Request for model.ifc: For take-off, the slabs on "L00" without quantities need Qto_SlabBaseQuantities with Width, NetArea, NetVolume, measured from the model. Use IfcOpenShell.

First a look at what the model holds.

```python
import ifcopenshell
import ifcopenshell.util.element
import ifcopenshell.util.unit

model = ifcopenshell.open("model.ifc")
print(model.schema)
for unit_type in ("LENGTHUNIT", "AREAUNIT", "VOLUMEUNIT"):
    print(unit_type, ifcopenshell.util.unit.calculate_unit_scale(model, unit_type))
storey = next(s for s in model.by_type("IfcBuildingStorey") if s.Name == "L00")
slabs = [e for e in ifcopenshell.util.element.get_decomposition(storey) if e.is_a("IfcSlab")]
for e in sorted(slabs, key=lambda e: e.id()):
    print(e.id(), e.is_a(), e.Name, list(ifcopenshell.util.element.get_psets(e, qtos_only=True)), sep=" | ")
```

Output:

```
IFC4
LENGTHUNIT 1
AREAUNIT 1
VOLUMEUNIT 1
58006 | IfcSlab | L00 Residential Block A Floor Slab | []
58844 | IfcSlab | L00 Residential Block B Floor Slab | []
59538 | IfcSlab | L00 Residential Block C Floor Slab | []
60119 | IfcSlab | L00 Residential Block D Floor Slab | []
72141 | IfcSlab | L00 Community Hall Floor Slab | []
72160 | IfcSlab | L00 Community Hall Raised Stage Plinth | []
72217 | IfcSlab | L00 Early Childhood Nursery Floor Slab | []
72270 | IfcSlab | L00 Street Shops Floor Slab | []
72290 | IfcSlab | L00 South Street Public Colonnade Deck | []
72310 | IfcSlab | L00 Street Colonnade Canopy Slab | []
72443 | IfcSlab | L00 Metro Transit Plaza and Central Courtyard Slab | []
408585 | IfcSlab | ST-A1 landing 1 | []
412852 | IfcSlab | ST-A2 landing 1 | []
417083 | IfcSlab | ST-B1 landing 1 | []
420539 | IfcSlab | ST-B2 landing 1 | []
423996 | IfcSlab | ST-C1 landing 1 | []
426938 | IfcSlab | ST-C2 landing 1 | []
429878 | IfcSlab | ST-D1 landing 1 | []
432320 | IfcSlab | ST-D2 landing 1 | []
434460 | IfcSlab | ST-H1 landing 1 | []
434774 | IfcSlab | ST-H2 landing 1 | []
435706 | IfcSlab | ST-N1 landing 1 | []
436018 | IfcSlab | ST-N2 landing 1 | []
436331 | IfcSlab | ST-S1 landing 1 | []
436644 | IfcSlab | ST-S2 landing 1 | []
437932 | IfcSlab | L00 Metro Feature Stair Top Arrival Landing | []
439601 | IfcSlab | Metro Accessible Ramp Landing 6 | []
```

```python
import ifcopenshell
import ifcopenshell.api.pset
import ifcopenshell.geom
import ifcopenshell.util.element
import ifcopenshell.util.shape
import ifcopenshell.util.unit

model = ifcopenshell.open("model.ifc")
unit_scale = ifcopenshell.util.unit.calculate_unit_scale(model)
area_scale = ifcopenshell.util.unit.calculate_unit_scale(model, "AREAUNIT")
volume_scale = ifcopenshell.util.unit.calculate_unit_scale(model, "VOLUMEUNIT")
settings = ifcopenshell.geom.settings()

storey = next(s for s in model.by_type("IfcBuildingStorey") if s.Name == "L00")
slabs = [e for e in ifcopenshell.util.element.get_decomposition(storey) if e.is_a("IfcSlab")]

for e in sorted(slabs, key=lambda e: e.id()):
    if ifcopenshell.util.element.get_psets(e, qtos_only=True, should_inherit=False):
        continue
    # Geometry comes back in metres, in the element's own axes.
    shape = ifcopenshell.geom.create_shape(settings, e)
    values = {
        "Width": ifcopenshell.util.shape.get_z(shape.geometry) / unit_scale,
        "NetArea": ifcopenshell.util.shape.get_footprint_area(shape.geometry) / area_scale,
        "NetVolume": ifcopenshell.util.shape.get_volume(shape.geometry) / volume_scale,
    }
    qto = ifcopenshell.api.pset.add_qto(model, product=e, name="Qto_SlabBaseQuantities")
    ifcopenshell.api.pset.edit_qto(model, qto=qto, properties=values)
    print(e.id(), {k: round(v, 3) for k, v in values.items()})

model.write("model_edited.ifc")
```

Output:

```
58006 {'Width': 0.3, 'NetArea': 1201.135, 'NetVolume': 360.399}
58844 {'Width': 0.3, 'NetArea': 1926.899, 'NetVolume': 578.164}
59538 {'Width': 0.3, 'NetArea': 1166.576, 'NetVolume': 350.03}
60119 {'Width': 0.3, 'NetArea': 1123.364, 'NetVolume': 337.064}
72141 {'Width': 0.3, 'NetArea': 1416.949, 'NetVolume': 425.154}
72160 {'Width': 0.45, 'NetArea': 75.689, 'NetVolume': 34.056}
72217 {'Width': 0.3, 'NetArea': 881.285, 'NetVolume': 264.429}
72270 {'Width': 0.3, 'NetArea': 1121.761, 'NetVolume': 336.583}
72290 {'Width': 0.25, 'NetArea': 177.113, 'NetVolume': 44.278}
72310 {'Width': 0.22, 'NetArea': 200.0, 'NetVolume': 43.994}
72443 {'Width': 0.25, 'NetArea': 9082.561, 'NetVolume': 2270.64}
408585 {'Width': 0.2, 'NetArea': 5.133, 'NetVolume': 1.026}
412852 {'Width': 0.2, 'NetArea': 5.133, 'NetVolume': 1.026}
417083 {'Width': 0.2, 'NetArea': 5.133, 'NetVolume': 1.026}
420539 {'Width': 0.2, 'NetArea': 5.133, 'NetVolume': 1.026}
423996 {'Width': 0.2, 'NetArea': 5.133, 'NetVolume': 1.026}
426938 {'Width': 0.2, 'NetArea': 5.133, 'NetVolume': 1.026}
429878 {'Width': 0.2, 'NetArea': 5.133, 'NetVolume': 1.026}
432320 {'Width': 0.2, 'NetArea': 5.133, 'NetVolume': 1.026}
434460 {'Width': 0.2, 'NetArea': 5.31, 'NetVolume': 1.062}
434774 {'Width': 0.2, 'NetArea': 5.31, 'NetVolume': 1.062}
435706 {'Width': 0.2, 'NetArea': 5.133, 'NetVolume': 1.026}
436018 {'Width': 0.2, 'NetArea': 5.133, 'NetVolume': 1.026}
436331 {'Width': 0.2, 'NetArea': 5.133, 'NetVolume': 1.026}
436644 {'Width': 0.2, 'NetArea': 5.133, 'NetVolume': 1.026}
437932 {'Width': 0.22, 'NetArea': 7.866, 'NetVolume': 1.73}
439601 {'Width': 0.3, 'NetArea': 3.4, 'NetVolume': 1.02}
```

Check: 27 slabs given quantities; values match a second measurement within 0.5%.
